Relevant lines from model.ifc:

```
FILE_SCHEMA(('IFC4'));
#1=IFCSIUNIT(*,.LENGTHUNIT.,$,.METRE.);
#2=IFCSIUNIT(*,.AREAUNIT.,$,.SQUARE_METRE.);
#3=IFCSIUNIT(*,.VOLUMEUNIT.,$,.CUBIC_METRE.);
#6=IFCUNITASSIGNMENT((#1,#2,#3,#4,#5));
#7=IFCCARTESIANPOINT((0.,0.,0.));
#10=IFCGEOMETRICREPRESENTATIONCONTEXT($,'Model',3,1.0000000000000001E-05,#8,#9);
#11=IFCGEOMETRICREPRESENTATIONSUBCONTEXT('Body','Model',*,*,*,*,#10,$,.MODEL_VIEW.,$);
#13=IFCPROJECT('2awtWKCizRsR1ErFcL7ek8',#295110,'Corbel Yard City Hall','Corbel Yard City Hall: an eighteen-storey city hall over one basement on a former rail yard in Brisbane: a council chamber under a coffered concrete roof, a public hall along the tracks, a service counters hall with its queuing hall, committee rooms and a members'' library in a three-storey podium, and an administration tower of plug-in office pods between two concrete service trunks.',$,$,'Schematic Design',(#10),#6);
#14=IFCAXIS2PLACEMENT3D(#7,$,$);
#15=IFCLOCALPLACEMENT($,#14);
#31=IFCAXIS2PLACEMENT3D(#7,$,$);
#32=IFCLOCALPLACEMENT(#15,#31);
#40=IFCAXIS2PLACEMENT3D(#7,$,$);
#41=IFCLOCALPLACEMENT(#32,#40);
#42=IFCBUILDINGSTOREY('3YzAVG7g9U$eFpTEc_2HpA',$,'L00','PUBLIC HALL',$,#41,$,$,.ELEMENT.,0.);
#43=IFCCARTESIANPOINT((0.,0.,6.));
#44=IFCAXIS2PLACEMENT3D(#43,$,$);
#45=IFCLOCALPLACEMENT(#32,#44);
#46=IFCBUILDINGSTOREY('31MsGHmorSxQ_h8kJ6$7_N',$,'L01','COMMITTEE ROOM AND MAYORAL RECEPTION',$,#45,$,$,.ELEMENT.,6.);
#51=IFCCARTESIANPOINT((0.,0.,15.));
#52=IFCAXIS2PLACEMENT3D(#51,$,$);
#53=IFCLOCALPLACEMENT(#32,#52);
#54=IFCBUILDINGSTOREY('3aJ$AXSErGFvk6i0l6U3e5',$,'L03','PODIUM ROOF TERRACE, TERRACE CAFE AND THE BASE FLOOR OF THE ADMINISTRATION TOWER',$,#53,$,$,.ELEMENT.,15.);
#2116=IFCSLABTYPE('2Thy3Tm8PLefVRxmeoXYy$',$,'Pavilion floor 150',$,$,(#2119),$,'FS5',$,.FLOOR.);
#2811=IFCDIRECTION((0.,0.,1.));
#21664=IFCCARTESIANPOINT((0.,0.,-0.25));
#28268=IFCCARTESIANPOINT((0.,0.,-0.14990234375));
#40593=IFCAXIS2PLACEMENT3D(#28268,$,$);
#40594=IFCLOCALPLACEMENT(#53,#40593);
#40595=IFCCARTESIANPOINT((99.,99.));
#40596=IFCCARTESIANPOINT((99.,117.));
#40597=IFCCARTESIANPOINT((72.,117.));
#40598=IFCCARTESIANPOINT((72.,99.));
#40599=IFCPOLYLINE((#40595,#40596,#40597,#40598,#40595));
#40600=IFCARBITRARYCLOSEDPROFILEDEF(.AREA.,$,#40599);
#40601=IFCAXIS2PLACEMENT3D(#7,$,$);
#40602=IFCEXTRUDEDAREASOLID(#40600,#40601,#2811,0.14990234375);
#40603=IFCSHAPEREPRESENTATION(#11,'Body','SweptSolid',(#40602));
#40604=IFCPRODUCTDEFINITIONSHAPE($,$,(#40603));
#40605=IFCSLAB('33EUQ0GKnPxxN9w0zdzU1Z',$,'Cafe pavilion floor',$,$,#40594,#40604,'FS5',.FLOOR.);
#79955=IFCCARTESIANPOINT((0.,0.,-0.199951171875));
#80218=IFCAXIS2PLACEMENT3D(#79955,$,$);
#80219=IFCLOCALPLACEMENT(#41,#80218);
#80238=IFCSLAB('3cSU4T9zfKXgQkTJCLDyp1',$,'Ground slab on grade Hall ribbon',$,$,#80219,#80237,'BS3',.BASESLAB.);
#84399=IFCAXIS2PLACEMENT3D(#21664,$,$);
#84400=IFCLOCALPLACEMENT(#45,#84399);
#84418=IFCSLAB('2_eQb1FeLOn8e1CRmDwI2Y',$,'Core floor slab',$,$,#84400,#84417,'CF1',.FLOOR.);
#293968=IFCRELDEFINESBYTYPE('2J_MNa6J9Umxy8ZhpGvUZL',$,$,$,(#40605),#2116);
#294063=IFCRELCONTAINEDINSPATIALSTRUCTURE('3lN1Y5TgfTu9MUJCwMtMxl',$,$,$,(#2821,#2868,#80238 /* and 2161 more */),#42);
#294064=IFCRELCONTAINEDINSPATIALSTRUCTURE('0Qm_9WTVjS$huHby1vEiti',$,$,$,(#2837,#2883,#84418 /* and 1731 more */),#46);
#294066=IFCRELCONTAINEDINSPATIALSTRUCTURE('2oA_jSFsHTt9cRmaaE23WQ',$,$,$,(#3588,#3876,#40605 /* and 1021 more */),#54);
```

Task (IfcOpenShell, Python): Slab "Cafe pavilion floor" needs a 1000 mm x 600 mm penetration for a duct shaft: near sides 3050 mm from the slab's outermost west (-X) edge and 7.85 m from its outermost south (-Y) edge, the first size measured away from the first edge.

```python
import numpy as np
import ifcopenshell
import ifcopenshell.api.feature
import ifcopenshell.api.geometry
import ifcopenshell.api.root
import ifcopenshell.geom
import ifcopenshell.util.placement
import ifcopenshell.util.representation
import ifcopenshell.util.shape
import ifcopenshell.util.unit

model = ifcopenshell.open("model.ifc")
unit_scale = ifcopenshell.util.unit.calculate_unit_scale(model)
settings = ifcopenshell.geom.settings()


def volume(element):
    """Net volume in cubic metres, openings subtracted."""
    shape = ifcopenshell.geom.create_shape(settings, element)
    return ifcopenshell.util.shape.get_volume(shape.geometry)


slab = model.by_guid("33EUQ0GKnPxxN9w0zdzU1Z")
before = volume(slab)

# Extent in the slab's own axes, in metres. The edges named are its -X and -Y sides.
slab_shape = ifcopenshell.geom.create_shape(settings, slab)
vertices = ifcopenshell.util.shape.get_vertices(slab_shape.geometry)
x_min, y_min, bottom = vertices.min(axis=0)
top = vertices[:, 2].max()

opening = ifcopenshell.api.root.create_entity(model, ifc_class="IfcOpeningElement", name="Duct shaft opening", predefined_type="OPENING")
context = ifcopenshell.util.representation.get_context(model, "Model", "Body", "MODEL_VIEW")
width, depth = 1, 0.6
outline = [(0.0, 0.0), (width, 0.0), (width, depth), (0.0, depth), (0.0, 0.0)]
# Overshoot both faces by 50 mm so the cut is clean.
shape = ifcopenshell.api.geometry.add_slab_representation(
    model, context=context, depth=top - bottom + 0.1, polyline=outline
)
ifcopenshell.api.geometry.assign_representation(model, product=opening, representation=shape)

matrix = ifcopenshell.util.placement.get_local_placement(slab.ObjectPlacement)
matrix[:, 3] = matrix @ np.append(np.array([x_min + 3.05, y_min + 7.85, bottom - 0.05]) / unit_scale, 1.0)
ifcopenshell.api.geometry.edit_object_placement(model, product=opening, matrix=matrix, is_si=False)
ifcopenshell.api.feature.add_feature(model, feature=opening, element=slab)

after = volume(slab)

print(f"slab volume {before:.3f} -> {after:.3f} m3")

model.write("model_updated.ifc")
```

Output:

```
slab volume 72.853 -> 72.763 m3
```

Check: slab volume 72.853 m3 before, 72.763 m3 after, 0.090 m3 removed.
